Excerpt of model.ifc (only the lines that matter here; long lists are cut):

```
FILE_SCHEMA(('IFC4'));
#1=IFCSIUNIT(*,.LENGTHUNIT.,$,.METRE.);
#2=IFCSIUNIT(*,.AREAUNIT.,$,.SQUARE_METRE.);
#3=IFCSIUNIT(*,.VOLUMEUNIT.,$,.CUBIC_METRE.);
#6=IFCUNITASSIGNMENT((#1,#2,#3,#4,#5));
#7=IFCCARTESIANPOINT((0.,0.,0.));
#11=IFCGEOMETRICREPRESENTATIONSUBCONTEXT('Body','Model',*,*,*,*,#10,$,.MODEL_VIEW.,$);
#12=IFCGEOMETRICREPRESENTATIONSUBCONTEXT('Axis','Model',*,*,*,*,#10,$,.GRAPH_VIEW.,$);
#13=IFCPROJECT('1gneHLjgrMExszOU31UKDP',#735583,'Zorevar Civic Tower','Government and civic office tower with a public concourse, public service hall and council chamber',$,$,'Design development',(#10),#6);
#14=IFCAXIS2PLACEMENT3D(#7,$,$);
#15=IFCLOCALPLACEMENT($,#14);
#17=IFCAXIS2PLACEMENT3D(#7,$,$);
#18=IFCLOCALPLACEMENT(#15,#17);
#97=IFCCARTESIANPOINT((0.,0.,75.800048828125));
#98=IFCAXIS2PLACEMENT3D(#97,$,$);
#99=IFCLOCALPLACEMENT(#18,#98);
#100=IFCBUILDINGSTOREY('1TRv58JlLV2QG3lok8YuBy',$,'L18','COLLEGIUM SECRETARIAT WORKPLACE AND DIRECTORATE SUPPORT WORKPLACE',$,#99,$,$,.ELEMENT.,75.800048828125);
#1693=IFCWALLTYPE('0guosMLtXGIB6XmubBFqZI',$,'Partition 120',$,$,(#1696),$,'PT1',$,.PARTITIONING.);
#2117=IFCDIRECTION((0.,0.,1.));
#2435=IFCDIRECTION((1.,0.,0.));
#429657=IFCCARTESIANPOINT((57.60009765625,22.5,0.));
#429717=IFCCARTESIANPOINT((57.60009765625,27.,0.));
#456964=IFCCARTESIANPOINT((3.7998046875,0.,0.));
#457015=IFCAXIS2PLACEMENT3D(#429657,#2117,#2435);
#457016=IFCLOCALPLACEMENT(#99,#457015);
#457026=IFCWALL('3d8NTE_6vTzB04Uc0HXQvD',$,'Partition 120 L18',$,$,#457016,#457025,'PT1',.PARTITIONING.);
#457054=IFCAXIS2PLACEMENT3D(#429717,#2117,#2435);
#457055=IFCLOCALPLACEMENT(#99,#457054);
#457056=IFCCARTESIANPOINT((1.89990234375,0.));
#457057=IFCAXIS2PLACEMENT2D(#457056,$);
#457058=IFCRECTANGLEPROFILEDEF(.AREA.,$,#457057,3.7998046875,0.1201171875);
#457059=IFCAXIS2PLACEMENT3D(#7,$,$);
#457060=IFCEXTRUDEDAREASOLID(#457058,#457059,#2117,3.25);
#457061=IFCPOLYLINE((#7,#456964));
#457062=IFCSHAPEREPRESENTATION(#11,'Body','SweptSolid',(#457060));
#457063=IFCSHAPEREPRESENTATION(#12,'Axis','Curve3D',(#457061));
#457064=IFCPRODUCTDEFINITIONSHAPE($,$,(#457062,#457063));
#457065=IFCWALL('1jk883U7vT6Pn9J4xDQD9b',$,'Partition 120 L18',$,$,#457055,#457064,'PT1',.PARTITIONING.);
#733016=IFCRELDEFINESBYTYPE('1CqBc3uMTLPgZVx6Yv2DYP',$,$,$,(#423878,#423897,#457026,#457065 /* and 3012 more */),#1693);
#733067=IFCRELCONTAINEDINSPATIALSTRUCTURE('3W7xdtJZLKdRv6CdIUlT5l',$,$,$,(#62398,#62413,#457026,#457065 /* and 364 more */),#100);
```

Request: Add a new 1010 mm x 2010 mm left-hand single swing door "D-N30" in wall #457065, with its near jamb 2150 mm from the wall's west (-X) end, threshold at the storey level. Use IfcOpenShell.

```python
import numpy as np
import ifcopenshell
import ifcopenshell.api.feature
import ifcopenshell.api.geometry
import ifcopenshell.api.root
import ifcopenshell.api.spatial
import ifcopenshell.geom
import ifcopenshell.util.element
import ifcopenshell.util.placement
import ifcopenshell.util.representation
import ifcopenshell.util.shape
import ifcopenshell.util.unit

model = ifcopenshell.open("model.ifc")
unit_scale = ifcopenshell.util.unit.calculate_unit_scale(model)
settings = ifcopenshell.geom.settings()


def volume(element):
    """Net volume in cubic metres, openings subtracted."""
    shape = ifcopenshell.geom.create_shape(settings, element)
    return ifcopenshell.util.shape.get_volume(shape.geometry)


wall = model.by_id(457065)
storey = ifcopenshell.util.element.get_container(wall, ifc_class="IfcBuildingStorey")
context = ifcopenshell.util.representation.get_context(model, "Model", "Body", "MODEL_VIEW")
before = volume(wall)

width, height, from_end, sill = 1.01, 2.01, 2.15, 0.0  # metres

# The wall runs along its own X axis, and the end named is its -X end.
wall_shape = ifcopenshell.geom.create_shape(settings, wall)
x, y, z = ifcopenshell.util.shape.get_vertices(wall_shape.geometry).T
start = x.min() + from_end
face, thickness = float(y.min()), float(y.max() - y.min())
wall_matrix = ifcopenshell.util.placement.get_local_placement(wall.ObjectPlacement)
level = ifcopenshell.util.placement.get_local_placement(storey.ObjectPlacement)[2, 3]


def in_wall(x, y):
    """Placement at x, y metres in the wall's axes, at sill height."""
    matrix = wall_matrix.copy()
    matrix[:, 3] = wall_matrix @ np.array([x / unit_scale, y / unit_scale, 0.0, 1.0])
    matrix[2, 3] = level + sill / unit_scale
    return matrix


# Opening: a box that overshoots both wall faces by 50 mm.
opening = ifcopenshell.api.root.create_entity(model, ifc_class="IfcOpeningElement", predefined_type="OPENING")
box = ifcopenshell.api.geometry.add_wall_representation(
    model, context=context, length=width, height=height, thickness=thickness + 0.1
)
ifcopenshell.api.geometry.assign_representation(model, product=opening, representation=box)
ifcopenshell.api.geometry.edit_object_placement(model, product=opening, matrix=in_wall(start, face - 0.05), is_si=False)
ifcopenshell.api.feature.add_feature(model, feature=opening, element=wall)

door = ifcopenshell.api.root.create_entity(model, ifc_class="IfcDoor", name="D-N30", predefined_type="DOOR")
door.OverallWidth, door.OverallHeight = width / unit_scale, height / unit_scale
door.OperationType = "SINGLE_SWING_LEFT"
body = ifcopenshell.api.geometry.add_door_representation(
    model,
    context=context,
    overall_width=door.OverallWidth,
    overall_height=door.OverallHeight,
    operation_type="SINGLE_SWING_LEFT",
    lining_properties={"LiningDepth": thickness / unit_scale, "ThresholdDepth": thickness / unit_scale},
)
ifcopenshell.api.geometry.assign_representation(model, product=door, representation=body)
ifcopenshell.api.spatial.assign_container(model, products=[door], relating_structure=storey)
ifcopenshell.api.feature.add_filling(model, opening=opening, element=door)

# The lining spans the wall, so the door starts at the wall face.
ifcopenshell.api.geometry.edit_object_placement(model, product=door, matrix=in_wall(start, face), is_si=False)

after = volume(wall)

print(f"wall volume {before:.3f} -> {after:.3f} m3")

model.write("model_updated.ifc")
```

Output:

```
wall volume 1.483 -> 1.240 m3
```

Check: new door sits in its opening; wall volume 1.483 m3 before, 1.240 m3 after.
